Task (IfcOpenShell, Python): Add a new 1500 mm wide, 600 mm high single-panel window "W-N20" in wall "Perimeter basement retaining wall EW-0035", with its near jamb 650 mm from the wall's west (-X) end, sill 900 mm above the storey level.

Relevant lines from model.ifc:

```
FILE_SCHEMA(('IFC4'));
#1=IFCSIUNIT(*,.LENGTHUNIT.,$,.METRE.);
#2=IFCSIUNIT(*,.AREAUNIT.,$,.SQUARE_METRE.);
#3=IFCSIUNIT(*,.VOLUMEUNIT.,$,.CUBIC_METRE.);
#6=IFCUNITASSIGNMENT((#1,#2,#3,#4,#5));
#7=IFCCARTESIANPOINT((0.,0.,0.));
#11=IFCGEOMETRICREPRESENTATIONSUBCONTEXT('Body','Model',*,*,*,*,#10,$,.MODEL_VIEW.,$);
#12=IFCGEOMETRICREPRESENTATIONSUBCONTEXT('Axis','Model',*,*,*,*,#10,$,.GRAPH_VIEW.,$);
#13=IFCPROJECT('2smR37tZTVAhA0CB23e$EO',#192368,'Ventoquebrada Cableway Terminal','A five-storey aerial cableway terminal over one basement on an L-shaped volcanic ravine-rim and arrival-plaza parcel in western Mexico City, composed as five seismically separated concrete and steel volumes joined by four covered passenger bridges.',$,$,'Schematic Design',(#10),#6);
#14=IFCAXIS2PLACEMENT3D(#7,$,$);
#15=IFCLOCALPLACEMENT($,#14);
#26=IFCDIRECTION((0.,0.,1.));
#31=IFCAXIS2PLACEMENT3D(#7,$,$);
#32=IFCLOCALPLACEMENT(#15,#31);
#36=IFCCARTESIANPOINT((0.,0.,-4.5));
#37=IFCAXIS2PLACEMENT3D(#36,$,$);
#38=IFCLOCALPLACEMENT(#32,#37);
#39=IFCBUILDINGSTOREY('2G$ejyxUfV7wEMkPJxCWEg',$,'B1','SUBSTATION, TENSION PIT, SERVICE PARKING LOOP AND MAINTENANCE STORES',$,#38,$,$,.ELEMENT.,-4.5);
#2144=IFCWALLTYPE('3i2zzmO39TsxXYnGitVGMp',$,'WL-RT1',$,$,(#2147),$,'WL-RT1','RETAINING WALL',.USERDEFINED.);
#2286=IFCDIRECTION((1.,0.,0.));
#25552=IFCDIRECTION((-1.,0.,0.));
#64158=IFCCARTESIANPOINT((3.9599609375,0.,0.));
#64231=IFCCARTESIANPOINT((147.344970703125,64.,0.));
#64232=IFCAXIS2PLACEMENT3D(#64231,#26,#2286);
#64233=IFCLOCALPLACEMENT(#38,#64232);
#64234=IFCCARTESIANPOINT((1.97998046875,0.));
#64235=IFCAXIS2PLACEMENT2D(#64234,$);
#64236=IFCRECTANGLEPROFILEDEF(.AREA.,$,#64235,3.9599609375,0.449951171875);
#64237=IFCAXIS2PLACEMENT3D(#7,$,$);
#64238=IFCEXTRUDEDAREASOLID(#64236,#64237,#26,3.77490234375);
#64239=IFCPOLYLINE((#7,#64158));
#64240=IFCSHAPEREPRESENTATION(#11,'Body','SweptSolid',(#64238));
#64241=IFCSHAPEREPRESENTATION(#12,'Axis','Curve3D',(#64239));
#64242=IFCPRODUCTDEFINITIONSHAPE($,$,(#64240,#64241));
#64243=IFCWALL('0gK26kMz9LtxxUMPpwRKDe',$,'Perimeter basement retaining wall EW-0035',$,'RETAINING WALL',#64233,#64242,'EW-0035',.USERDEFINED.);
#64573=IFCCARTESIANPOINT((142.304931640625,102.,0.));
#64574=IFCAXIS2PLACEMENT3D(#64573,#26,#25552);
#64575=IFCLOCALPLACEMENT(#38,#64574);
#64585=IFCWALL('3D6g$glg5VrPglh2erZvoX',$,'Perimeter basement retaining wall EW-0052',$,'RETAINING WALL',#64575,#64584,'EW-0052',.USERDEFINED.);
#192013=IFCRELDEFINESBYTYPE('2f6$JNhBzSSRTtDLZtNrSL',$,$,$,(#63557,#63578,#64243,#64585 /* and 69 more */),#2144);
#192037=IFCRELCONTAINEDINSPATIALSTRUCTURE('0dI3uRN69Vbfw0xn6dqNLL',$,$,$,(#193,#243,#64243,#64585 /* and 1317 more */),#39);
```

```python
import numpy as np
import ifcopenshell
import ifcopenshell.api.feature
import ifcopenshell.api.geometry
import ifcopenshell.api.root
import ifcopenshell.api.spatial
import ifcopenshell.geom
import ifcopenshell.util.element
import ifcopenshell.util.placement
import ifcopenshell.util.representation
import ifcopenshell.util.shape
import ifcopenshell.util.unit

model = ifcopenshell.open("model.ifc")
unit_scale = ifcopenshell.util.unit.calculate_unit_scale(model)
settings = ifcopenshell.geom.settings()


def volume(element):
    """Net volume in cubic metres, openings subtracted."""
    shape = ifcopenshell.geom.create_shape(settings, element)
    return ifcopenshell.util.shape.get_volume(shape.geometry)


wall = model.by_id(64243)
storey = ifcopenshell.util.element.get_container(wall, ifc_class="IfcBuildingStorey")
context = ifcopenshell.util.representation.get_context(model, "Model", "Body", "MODEL_VIEW")
before = volume(wall)

width, height, from_end, sill = 1.5, 0.6, 0.65, 0.9  # metres

# The wall runs along its own X axis, and the end named is its -X end.
wall_shape = ifcopenshell.geom.create_shape(settings, wall)
x, y, z = ifcopenshell.util.shape.get_vertices(wall_shape.geometry).T
start = x.min() + from_end
face, thickness = float(y.min()), float(y.max() - y.min())
wall_matrix = ifcopenshell.util.placement.get_local_placement(wall.ObjectPlacement)
level = ifcopenshell.util.placement.get_local_placement(storey.ObjectPlacement)[2, 3]


def in_wall(x, y):
    """Placement at x, y metres in the wall's axes, at sill height."""
    matrix = wall_matrix.copy()
    matrix[:, 3] = wall_matrix @ np.array([x / unit_scale, y / unit_scale, 0.0, 1.0])
    matrix[2, 3] = level + sill / unit_scale
    return matrix


# Opening: a box that overshoots both wall faces by 50 mm.
opening = ifcopenshell.api.root.create_entity(model, ifc_class="IfcOpeningElement", predefined_type="OPENING")
box = ifcopenshell.api.geometry.add_wall_representation(
    model, context=context, length=width, height=height, thickness=thickness + 0.1
)
ifcopenshell.api.geometry.assign_representation(model, product=opening, representation=box)
ifcopenshell.api.geometry.edit_object_placement(model, product=opening, matrix=in_wall(start, face - 0.05), is_si=False)
ifcopenshell.api.feature.add_feature(model, feature=opening, element=wall)

window = ifcopenshell.api.root.create_entity(model, ifc_class="IfcWindow", name="W-N20", predefined_type="WINDOW")
window.OverallWidth, window.OverallHeight = width / unit_scale, height / unit_scale
window.PartitioningType = "SINGLE_PANEL"
body = ifcopenshell.api.geometry.add_window_representation(
    model,
    context=context,
    overall_width=window.OverallWidth,
    overall_height=window.OverallHeight,
    partition_type="SINGLE_PANEL",
)
ifcopenshell.api.geometry.assign_representation(model, product=window, representation=body)
ifcopenshell.api.spatial.assign_container(model, products=[window], relating_structure=storey)
ifcopenshell.api.feature.add_filling(model, opening=opening, element=window)

# Centre the window in the wall's thickness.
ifcopenshell.api.geometry.edit_object_placement(model, product=window, matrix=in_wall(start, face), is_si=False)
window_shape = ifcopenshell.geom.create_shape(settings, window)
depth = ifcopenshell.util.shape.get_vertices(window_shape.geometry)[:, 1]
offset = face + thickness / 2 - (depth.min() + depth.max()) / 2
ifcopenshell.api.geometry.edit_object_placement(model, product=window, matrix=in_wall(start, offset), is_si=False)

after = volume(wall)

print(f"wall volume {before:.3f} -> {after:.3f} m3")

model.write("model_v2.ifc")
```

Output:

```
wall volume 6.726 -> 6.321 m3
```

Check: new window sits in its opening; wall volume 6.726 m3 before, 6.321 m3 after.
